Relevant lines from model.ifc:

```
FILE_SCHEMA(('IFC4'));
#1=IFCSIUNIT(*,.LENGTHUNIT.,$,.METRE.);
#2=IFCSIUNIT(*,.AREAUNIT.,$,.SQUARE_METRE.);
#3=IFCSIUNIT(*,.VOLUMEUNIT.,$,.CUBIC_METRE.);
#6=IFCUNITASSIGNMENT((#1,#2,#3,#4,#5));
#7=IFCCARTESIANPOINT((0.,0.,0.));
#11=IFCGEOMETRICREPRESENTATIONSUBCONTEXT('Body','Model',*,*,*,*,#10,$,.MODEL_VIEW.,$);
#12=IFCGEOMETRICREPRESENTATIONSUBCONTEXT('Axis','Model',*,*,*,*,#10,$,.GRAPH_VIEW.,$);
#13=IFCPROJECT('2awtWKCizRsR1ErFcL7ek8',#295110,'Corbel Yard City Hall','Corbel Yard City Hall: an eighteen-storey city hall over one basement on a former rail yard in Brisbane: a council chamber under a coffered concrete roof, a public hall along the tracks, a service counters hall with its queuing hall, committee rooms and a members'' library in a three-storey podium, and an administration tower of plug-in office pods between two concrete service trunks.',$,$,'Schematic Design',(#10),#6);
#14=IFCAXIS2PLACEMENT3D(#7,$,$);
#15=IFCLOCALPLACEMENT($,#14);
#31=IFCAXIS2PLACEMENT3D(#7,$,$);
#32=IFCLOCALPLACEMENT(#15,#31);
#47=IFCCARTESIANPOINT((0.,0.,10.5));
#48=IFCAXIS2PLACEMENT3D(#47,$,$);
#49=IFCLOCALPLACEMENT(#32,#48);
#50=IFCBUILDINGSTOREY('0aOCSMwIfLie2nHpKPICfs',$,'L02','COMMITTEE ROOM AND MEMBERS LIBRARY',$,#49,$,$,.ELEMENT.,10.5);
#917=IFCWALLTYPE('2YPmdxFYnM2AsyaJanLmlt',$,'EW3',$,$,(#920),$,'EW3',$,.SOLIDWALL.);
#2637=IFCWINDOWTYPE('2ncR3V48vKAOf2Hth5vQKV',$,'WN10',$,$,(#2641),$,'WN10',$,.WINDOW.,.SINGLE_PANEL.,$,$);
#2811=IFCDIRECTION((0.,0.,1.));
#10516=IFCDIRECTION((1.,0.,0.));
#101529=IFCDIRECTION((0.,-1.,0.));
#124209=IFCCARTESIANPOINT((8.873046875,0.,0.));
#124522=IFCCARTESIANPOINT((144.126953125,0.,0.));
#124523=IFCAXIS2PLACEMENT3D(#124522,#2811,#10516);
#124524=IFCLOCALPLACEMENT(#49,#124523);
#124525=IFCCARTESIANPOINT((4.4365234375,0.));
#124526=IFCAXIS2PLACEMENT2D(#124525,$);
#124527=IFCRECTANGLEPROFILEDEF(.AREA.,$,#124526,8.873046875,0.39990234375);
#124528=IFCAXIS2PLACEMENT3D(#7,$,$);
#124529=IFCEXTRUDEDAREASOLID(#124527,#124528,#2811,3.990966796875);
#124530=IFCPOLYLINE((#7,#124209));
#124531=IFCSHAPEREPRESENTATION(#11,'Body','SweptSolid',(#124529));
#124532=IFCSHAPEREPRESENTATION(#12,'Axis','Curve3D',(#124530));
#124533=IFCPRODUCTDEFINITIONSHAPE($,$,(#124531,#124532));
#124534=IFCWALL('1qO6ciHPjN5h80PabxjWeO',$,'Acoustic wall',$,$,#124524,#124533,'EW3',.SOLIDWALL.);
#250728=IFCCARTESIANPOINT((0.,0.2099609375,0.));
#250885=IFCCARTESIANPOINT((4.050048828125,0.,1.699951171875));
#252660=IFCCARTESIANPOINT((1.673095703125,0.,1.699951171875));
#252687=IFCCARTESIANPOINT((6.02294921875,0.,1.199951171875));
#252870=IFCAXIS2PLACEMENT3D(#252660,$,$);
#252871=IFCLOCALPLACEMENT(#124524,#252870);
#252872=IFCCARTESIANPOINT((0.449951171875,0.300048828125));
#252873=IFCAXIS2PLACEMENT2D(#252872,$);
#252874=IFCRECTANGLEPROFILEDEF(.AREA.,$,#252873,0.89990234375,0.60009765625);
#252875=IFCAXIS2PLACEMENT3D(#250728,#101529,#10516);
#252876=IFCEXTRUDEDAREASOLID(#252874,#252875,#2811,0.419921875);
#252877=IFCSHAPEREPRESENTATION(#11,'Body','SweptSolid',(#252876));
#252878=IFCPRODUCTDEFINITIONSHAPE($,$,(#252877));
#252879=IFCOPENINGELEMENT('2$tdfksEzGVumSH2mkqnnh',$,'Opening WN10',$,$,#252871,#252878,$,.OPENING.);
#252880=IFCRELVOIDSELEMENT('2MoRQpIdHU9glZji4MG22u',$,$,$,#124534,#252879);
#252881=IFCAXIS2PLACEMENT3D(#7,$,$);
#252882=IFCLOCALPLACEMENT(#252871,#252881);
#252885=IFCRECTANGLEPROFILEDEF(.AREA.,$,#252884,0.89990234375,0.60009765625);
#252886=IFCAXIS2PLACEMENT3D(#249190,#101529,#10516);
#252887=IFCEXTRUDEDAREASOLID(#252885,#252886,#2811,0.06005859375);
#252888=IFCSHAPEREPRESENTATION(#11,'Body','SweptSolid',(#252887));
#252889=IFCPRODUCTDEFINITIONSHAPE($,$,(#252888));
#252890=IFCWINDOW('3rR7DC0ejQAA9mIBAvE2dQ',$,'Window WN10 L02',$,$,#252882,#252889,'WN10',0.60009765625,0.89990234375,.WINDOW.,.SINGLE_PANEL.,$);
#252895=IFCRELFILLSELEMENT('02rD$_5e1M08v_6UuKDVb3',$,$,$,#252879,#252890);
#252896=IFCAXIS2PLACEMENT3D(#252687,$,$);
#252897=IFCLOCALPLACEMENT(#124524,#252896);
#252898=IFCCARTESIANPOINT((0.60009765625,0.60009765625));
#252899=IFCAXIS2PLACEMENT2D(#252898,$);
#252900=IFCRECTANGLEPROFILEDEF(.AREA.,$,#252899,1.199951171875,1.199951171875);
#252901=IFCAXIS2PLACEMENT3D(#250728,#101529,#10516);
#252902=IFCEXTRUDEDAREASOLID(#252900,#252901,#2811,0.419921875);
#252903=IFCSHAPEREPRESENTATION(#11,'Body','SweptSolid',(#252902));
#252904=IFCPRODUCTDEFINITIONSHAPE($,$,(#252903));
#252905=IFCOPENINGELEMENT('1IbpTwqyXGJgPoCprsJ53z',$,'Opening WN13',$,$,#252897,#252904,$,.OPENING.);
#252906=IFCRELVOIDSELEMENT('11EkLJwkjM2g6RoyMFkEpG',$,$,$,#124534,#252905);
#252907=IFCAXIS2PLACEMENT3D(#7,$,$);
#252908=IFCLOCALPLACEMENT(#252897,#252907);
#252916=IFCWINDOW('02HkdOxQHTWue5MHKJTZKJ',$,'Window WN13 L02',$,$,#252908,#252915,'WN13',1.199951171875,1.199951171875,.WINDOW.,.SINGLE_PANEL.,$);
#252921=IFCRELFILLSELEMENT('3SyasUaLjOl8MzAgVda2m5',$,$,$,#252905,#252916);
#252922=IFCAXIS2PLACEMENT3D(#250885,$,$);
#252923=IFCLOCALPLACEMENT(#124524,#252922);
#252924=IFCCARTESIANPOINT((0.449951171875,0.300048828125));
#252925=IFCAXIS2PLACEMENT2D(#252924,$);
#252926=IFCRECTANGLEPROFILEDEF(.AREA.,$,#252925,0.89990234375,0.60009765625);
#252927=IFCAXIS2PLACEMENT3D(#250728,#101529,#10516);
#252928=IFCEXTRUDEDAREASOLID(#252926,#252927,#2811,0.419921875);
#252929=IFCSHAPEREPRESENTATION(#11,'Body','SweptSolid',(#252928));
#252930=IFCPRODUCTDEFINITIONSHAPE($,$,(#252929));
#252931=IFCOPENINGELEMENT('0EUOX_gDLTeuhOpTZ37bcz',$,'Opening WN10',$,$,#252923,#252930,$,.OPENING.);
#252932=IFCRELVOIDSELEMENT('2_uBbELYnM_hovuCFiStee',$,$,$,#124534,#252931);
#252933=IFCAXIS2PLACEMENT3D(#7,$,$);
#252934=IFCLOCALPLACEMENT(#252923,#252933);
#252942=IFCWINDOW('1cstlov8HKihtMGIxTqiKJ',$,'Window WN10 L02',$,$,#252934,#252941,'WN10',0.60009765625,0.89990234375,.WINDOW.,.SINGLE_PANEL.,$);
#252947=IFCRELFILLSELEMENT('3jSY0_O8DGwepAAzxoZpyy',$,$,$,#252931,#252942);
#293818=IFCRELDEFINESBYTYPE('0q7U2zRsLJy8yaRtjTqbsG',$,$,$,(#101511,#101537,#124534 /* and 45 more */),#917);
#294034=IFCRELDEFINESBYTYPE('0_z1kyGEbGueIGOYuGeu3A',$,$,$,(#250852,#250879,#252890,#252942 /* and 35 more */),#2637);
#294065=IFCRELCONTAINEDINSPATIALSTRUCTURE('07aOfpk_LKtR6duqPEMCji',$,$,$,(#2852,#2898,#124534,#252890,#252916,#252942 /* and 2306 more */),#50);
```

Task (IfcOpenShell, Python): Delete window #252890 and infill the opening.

```python
import ifcopenshell
import ifcopenshell.api.feature
import ifcopenshell.api.root
import ifcopenshell.geom
import ifcopenshell.util.shape

model = ifcopenshell.open("model.ifc")
settings = ifcopenshell.geom.settings()


def volume(element):
    """Net volume in cubic metres, openings subtracted."""
    shape = ifcopenshell.geom.create_shape(settings, element)
    return ifcopenshell.util.shape.get_volume(shape.geometry)


window = model.by_guid("3rR7DC0ejQAA9mIBAvE2dQ")
opening = window.FillsVoids[0].RelatingOpeningElement
wall = opening.VoidsElements[0].RelatingBuildingElement
before = volume(wall)

ifcopenshell.api.root.remove_product(model, product=window)
ifcopenshell.api.feature.remove_feature(model, feature=opening)

after = volume(wall)

print(f"wall volume {before:.3f} -> {after:.3f} m3")

model.write("model_v2.ifc")
```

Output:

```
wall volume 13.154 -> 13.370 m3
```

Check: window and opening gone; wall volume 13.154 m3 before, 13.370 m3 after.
